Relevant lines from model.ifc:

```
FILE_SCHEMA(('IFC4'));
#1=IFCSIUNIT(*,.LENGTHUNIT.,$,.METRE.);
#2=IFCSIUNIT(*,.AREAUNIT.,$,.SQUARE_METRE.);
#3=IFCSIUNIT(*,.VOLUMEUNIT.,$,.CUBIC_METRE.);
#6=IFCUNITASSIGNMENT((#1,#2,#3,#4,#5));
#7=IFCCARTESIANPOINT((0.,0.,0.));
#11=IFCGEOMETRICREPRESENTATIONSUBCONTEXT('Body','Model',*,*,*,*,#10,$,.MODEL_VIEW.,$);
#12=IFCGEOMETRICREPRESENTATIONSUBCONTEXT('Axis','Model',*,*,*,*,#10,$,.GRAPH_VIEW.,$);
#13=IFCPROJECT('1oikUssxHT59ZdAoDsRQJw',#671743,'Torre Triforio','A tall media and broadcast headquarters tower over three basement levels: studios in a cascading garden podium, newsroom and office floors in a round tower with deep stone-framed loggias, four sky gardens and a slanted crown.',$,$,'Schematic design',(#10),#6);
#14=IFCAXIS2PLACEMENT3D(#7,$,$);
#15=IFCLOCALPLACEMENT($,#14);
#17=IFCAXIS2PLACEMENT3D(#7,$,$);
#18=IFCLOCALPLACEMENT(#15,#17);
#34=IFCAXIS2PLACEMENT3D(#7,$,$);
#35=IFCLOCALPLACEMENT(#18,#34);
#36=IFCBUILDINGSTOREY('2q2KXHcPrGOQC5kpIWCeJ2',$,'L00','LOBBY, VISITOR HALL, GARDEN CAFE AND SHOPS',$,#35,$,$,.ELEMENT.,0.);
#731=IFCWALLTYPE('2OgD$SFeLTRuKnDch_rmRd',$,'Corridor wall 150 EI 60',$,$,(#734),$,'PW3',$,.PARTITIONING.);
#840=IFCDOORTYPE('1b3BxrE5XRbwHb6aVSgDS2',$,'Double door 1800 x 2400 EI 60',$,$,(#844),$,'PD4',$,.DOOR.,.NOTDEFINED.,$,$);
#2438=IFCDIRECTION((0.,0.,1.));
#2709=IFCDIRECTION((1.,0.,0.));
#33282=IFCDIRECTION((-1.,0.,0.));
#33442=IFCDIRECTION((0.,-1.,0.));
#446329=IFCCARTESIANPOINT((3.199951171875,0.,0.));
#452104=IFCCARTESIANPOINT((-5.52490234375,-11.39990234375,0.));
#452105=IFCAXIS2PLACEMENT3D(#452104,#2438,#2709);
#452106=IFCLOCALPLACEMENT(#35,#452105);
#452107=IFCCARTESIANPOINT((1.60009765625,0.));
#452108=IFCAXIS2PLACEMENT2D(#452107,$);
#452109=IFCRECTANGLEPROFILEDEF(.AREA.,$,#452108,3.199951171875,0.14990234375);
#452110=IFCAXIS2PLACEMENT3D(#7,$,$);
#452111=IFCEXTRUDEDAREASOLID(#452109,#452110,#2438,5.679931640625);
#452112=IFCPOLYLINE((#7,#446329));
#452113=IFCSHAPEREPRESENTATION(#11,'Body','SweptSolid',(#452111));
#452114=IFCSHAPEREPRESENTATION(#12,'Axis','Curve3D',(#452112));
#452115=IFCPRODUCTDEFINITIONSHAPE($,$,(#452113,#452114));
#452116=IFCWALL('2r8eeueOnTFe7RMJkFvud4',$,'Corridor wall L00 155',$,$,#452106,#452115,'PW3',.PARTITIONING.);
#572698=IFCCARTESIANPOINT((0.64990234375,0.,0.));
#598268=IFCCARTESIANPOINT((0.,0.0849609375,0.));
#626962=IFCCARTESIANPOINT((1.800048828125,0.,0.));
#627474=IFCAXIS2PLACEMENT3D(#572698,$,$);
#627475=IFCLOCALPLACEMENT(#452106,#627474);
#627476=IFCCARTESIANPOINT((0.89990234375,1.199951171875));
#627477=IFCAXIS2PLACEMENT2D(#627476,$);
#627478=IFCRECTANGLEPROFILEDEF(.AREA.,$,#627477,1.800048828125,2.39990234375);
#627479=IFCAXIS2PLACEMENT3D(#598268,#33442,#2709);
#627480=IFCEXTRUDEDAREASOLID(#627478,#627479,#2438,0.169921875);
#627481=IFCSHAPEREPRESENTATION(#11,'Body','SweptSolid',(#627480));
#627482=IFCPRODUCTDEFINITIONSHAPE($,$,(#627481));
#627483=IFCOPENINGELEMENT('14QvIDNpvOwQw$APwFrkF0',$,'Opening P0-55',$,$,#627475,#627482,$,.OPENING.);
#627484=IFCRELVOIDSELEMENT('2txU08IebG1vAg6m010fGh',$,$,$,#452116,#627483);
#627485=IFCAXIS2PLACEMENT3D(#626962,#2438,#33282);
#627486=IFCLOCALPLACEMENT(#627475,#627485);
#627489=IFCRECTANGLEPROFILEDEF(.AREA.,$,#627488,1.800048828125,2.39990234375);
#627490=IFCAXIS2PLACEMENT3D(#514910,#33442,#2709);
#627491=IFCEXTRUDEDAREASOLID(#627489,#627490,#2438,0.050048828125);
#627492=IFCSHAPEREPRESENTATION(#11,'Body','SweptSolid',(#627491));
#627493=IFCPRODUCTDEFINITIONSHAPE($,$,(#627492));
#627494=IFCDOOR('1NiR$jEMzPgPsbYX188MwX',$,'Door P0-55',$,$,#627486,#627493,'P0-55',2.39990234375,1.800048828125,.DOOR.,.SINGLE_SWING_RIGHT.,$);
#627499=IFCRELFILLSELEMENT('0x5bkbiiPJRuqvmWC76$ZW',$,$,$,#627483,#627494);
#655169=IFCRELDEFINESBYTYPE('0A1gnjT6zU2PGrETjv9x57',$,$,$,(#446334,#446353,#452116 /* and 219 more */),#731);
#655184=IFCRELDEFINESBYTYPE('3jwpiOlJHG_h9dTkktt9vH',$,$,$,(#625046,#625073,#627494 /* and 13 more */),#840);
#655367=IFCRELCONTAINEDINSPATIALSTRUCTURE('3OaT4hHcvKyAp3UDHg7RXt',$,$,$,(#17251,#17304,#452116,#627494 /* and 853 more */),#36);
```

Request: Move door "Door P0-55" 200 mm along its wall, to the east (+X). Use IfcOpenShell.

```python
import ifcopenshell
import ifcopenshell.api.geometry
import ifcopenshell.util.placement

model = ifcopenshell.open("model.ifc")

door = model.by_guid("1NiR$jEMzPgPsbYX188MwX")
opening = door.FillsVoids[0].RelatingOpeningElement
wall = opening.VoidsElements[0].RelatingBuildingElement

wall_matrix = ifcopenshell.util.placement.get_local_placement(wall.ObjectPlacement)
shift = wall_matrix[:3, 0] * 0.2
before = ifcopenshell.util.placement.get_local_placement(door.ObjectPlacement)[:3, 3].copy()

# The door is placed relative to its opening, so it follows when the opening moves.
matrix = ifcopenshell.util.placement.get_local_placement(opening.ObjectPlacement)
matrix[:3, 3] += shift
ifcopenshell.api.geometry.edit_object_placement(
    model, product=opening, matrix=matrix, is_si=False, should_transform_children=True
)

after = ifcopenshell.util.placement.get_local_placement(door.ObjectPlacement)[:3, 3]
print("door moved by", (after - before).round(3) + 0.0)

model.write("model_updated.ifc")
```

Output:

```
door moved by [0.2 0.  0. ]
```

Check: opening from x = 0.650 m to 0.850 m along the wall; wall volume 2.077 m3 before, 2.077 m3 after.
